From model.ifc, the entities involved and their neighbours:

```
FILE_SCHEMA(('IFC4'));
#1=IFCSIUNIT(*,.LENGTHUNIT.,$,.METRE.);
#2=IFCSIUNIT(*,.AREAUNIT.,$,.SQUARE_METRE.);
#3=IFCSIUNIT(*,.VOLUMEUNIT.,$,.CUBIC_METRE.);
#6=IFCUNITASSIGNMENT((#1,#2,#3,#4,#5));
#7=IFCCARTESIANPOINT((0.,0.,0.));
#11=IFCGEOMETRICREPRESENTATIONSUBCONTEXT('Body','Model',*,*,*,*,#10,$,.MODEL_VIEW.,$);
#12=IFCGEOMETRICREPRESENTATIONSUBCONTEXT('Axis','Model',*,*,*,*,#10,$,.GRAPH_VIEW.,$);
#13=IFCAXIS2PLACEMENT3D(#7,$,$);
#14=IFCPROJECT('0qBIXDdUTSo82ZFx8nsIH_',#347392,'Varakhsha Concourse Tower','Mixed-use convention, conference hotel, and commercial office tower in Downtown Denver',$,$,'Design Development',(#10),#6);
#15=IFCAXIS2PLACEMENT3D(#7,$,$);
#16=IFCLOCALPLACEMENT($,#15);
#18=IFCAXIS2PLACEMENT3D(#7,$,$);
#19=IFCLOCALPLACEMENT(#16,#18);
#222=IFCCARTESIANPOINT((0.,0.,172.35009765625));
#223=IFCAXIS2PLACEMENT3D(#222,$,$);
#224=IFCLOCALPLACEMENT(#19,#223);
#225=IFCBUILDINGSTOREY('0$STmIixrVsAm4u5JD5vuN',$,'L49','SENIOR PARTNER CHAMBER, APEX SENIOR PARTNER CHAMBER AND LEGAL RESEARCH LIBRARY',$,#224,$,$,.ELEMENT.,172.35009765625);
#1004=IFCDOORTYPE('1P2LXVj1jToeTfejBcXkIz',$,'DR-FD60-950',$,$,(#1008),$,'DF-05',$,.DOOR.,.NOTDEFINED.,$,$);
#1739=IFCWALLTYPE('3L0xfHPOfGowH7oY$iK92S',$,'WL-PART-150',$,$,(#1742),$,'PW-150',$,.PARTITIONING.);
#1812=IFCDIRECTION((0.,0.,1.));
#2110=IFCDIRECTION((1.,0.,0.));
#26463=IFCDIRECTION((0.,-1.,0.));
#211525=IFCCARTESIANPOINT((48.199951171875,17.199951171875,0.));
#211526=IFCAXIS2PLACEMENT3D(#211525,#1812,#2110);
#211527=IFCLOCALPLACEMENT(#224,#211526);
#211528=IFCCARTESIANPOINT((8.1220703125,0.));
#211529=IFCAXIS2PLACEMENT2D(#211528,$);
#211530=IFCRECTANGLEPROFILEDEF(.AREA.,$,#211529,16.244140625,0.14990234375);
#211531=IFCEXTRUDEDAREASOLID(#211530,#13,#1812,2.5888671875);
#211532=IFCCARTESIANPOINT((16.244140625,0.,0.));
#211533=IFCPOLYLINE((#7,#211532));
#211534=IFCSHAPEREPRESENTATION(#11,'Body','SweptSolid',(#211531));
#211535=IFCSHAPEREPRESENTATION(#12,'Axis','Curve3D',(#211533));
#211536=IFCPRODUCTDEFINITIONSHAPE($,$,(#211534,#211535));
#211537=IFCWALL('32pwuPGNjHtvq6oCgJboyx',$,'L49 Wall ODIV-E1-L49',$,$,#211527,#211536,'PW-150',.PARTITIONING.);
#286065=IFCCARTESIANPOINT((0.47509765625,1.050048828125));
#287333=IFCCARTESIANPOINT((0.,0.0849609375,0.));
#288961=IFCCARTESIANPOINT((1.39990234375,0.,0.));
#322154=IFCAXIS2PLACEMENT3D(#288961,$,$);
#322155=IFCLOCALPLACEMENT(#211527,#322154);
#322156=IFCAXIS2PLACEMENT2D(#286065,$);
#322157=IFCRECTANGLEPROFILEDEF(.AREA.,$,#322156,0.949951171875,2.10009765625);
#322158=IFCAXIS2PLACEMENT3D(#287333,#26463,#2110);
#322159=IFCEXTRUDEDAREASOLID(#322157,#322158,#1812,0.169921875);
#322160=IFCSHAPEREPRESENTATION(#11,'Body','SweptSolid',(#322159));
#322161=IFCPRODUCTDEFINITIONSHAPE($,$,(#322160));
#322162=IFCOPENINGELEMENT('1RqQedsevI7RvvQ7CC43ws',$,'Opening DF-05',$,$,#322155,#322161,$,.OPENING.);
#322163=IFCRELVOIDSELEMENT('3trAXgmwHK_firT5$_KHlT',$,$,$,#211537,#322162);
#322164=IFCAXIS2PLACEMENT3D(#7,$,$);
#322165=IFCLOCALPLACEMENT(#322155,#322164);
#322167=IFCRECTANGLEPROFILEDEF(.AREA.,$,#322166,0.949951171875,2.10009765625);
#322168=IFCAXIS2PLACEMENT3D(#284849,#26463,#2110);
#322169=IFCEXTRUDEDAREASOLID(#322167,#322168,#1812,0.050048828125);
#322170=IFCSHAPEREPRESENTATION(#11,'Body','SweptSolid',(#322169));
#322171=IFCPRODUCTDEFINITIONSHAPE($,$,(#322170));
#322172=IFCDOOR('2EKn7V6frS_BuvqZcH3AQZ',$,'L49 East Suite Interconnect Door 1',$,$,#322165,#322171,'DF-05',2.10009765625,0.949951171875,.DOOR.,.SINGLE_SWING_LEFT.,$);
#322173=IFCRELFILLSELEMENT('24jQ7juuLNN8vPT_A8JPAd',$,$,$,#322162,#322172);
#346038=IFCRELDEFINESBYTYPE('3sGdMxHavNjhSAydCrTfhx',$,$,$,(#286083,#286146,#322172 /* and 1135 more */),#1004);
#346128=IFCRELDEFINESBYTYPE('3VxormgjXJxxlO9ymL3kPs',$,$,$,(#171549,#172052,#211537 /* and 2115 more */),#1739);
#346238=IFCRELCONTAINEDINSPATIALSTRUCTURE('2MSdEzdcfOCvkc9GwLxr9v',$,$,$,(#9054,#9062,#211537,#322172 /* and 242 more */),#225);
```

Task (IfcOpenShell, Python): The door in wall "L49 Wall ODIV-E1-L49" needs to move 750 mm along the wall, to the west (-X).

```python
import ifcopenshell
import ifcopenshell.api.geometry
import ifcopenshell.util.placement

model = ifcopenshell.open("model.ifc")

door = model.by_guid("2EKn7V6frS_BuvqZcH3AQZ")
opening = door.FillsVoids[0].RelatingOpeningElement
wall = opening.VoidsElements[0].RelatingBuildingElement

wall_matrix = ifcopenshell.util.placement.get_local_placement(wall.ObjectPlacement)
shift = wall_matrix[:3, 0] * -0.75
before = ifcopenshell.util.placement.get_local_placement(door.ObjectPlacement)[:3, 3].copy()

# The door is placed relative to its opening, so it follows when the opening moves.
matrix = ifcopenshell.util.placement.get_local_placement(opening.ObjectPlacement)
matrix[:3, 3] += shift
ifcopenshell.api.geometry.edit_object_placement(
    model, product=opening, matrix=matrix, is_si=False, should_transform_children=True
)

after = ifcopenshell.util.placement.get_local_placement(door.ObjectPlacement)[:3, 3]
print("door moved by", (after - before).round(3) + 0.0)

model.write("model_edited.ifc")
```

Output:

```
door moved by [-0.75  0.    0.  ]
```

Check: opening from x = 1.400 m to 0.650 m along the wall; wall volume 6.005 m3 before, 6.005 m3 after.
